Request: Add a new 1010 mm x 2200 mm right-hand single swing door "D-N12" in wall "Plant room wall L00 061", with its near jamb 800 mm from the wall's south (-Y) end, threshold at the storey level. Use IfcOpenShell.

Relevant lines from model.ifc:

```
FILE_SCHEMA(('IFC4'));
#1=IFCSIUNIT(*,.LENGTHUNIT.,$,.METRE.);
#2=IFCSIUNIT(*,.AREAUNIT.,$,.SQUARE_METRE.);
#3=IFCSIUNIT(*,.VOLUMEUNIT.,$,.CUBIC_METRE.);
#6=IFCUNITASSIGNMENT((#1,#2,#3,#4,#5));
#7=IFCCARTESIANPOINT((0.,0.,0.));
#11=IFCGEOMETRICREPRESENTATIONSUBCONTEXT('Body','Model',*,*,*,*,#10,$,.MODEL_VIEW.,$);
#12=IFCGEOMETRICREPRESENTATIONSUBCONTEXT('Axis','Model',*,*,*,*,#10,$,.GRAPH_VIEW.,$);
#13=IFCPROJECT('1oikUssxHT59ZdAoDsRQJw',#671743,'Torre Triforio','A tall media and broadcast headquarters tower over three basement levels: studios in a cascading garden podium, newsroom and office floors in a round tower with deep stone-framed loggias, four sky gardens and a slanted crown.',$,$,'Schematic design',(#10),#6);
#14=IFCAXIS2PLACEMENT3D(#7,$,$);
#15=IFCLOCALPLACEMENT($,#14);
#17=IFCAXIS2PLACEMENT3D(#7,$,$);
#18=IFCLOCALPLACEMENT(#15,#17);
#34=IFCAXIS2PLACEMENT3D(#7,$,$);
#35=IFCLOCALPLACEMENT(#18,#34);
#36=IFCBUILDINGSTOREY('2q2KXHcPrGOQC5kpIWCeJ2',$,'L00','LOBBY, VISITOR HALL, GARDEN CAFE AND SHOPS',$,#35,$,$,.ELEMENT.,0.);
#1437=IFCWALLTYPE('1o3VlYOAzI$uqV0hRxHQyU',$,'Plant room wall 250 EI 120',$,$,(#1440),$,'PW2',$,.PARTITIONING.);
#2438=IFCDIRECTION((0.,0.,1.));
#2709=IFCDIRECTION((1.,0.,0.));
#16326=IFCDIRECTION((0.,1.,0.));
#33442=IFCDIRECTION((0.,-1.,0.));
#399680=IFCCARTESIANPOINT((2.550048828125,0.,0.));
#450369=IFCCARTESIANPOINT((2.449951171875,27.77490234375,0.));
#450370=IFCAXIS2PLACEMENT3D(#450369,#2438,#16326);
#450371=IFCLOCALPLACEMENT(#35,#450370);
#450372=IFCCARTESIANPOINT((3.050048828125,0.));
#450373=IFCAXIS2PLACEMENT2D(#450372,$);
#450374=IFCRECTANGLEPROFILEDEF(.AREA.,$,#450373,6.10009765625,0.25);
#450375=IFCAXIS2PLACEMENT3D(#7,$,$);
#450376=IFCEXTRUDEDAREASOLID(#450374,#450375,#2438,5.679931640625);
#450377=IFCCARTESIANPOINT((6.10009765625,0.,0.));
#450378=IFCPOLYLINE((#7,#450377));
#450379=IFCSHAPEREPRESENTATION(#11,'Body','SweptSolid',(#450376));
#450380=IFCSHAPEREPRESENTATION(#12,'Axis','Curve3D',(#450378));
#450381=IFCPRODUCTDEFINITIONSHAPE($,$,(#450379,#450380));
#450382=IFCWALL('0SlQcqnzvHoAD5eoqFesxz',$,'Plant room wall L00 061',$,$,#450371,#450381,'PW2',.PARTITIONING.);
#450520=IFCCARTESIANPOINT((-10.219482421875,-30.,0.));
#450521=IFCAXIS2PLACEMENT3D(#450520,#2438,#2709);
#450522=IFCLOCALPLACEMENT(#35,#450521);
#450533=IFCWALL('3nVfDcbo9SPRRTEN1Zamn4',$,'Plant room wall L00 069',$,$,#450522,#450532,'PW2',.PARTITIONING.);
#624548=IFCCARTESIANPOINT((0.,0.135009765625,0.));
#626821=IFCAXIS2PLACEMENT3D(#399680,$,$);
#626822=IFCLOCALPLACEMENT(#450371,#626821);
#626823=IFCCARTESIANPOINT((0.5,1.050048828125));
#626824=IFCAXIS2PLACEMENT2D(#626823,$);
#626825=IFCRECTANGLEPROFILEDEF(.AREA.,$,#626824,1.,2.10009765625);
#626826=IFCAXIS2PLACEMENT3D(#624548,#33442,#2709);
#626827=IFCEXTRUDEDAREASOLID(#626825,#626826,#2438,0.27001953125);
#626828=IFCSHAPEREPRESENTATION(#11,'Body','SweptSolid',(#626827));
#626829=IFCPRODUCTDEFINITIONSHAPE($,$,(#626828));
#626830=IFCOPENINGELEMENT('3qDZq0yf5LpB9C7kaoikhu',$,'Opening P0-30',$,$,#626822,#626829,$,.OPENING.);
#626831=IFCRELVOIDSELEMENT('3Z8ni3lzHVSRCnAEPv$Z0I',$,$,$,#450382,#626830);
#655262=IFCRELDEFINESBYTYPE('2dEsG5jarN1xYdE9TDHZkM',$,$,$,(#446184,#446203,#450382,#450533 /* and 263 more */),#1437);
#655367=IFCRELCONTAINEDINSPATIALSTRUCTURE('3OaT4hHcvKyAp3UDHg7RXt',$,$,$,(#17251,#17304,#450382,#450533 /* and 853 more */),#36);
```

```python
import numpy as np
import ifcopenshell
import ifcopenshell.api.feature
import ifcopenshell.api.geometry
import ifcopenshell.api.root
import ifcopenshell.api.spatial
import ifcopenshell.geom
import ifcopenshell.util.element
import ifcopenshell.util.placement
import ifcopenshell.util.representation
import ifcopenshell.util.shape
import ifcopenshell.util.unit

model = ifcopenshell.open("model.ifc")
unit_scale = ifcopenshell.util.unit.calculate_unit_scale(model)
settings = ifcopenshell.geom.settings()


def volume(element):
    """Net volume in cubic metres, openings subtracted."""
    shape = ifcopenshell.geom.create_shape(settings, element)
    return ifcopenshell.util.shape.get_volume(shape.geometry)


wall = model.by_guid("0SlQcqnzvHoAD5eoqFesxz")
storey = ifcopenshell.util.element.get_container(wall, ifc_class="IfcBuildingStorey")
context = ifcopenshell.util.representation.get_context(model, "Model", "Body", "MODEL_VIEW")
before = volume(wall)

width, height, from_end, sill = 1.01, 2.2, 0.8, 0.0  # metres

# The wall runs along its own X axis, and the end named is its -X end.
wall_shape = ifcopenshell.geom.create_shape(settings, wall)
x, y, z = ifcopenshell.util.shape.get_vertices(wall_shape.geometry).T
start = x.min() + from_end
face, thickness = float(y.min()), float(y.max() - y.min())
wall_matrix = ifcopenshell.util.placement.get_local_placement(wall.ObjectPlacement)
level = ifcopenshell.util.placement.get_local_placement(storey.ObjectPlacement)[2, 3]


def in_wall(x, y):
    """Placement at x, y metres in the wall's axes, at sill height."""
    matrix = wall_matrix.copy()
    matrix[:, 3] = wall_matrix @ np.array([x / unit_scale, y / unit_scale, 0.0, 1.0])
    matrix[2, 3] = level + sill / unit_scale
    return matrix


# Opening: a box that overshoots both wall faces by 50 mm.
opening = ifcopenshell.api.root.create_entity(model, ifc_class="IfcOpeningElement", predefined_type="OPENING")
box = ifcopenshell.api.geometry.add_wall_representation(
    model, context=context, length=width, height=height, thickness=thickness + 0.1
)
ifcopenshell.api.geometry.assign_representation(model, product=opening, representation=box)
ifcopenshell.api.geometry.edit_object_placement(model, product=opening, matrix=in_wall(start, face - 0.05), is_si=False)
ifcopenshell.api.feature.add_feature(model, feature=opening, element=wall)

door = ifcopenshell.api.root.create_entity(model, ifc_class="IfcDoor", name="D-N12", predefined_type="DOOR")
door.OverallWidth, door.OverallHeight = width / unit_scale, height / unit_scale
door.OperationType = "SINGLE_SWING_RIGHT"
body = ifcopenshell.api.geometry.add_door_representation(
    model,
    context=context,
    overall_width=door.OverallWidth,
    overall_height=door.OverallHeight,
    operation_type="SINGLE_SWING_RIGHT",
    lining_properties={"LiningDepth": thickness / unit_scale, "ThresholdDepth": thickness / unit_scale},
)
ifcopenshell.api.geometry.assign_representation(model, product=door, representation=body)
ifcopenshell.api.spatial.assign_container(model, products=[door], relating_structure=storey)
ifcopenshell.api.feature.add_filling(model, opening=opening, element=door)

# The lining spans the wall, so the door starts at the wall face.
ifcopenshell.api.geometry.edit_object_placement(model, product=door, matrix=in_wall(start, face), is_si=False)

after = volume(wall)

print(f"wall volume {before:.3f} -> {after:.3f} m3")

model.write("model_rev.ifc")
```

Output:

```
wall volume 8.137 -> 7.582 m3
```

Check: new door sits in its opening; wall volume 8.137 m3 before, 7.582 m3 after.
